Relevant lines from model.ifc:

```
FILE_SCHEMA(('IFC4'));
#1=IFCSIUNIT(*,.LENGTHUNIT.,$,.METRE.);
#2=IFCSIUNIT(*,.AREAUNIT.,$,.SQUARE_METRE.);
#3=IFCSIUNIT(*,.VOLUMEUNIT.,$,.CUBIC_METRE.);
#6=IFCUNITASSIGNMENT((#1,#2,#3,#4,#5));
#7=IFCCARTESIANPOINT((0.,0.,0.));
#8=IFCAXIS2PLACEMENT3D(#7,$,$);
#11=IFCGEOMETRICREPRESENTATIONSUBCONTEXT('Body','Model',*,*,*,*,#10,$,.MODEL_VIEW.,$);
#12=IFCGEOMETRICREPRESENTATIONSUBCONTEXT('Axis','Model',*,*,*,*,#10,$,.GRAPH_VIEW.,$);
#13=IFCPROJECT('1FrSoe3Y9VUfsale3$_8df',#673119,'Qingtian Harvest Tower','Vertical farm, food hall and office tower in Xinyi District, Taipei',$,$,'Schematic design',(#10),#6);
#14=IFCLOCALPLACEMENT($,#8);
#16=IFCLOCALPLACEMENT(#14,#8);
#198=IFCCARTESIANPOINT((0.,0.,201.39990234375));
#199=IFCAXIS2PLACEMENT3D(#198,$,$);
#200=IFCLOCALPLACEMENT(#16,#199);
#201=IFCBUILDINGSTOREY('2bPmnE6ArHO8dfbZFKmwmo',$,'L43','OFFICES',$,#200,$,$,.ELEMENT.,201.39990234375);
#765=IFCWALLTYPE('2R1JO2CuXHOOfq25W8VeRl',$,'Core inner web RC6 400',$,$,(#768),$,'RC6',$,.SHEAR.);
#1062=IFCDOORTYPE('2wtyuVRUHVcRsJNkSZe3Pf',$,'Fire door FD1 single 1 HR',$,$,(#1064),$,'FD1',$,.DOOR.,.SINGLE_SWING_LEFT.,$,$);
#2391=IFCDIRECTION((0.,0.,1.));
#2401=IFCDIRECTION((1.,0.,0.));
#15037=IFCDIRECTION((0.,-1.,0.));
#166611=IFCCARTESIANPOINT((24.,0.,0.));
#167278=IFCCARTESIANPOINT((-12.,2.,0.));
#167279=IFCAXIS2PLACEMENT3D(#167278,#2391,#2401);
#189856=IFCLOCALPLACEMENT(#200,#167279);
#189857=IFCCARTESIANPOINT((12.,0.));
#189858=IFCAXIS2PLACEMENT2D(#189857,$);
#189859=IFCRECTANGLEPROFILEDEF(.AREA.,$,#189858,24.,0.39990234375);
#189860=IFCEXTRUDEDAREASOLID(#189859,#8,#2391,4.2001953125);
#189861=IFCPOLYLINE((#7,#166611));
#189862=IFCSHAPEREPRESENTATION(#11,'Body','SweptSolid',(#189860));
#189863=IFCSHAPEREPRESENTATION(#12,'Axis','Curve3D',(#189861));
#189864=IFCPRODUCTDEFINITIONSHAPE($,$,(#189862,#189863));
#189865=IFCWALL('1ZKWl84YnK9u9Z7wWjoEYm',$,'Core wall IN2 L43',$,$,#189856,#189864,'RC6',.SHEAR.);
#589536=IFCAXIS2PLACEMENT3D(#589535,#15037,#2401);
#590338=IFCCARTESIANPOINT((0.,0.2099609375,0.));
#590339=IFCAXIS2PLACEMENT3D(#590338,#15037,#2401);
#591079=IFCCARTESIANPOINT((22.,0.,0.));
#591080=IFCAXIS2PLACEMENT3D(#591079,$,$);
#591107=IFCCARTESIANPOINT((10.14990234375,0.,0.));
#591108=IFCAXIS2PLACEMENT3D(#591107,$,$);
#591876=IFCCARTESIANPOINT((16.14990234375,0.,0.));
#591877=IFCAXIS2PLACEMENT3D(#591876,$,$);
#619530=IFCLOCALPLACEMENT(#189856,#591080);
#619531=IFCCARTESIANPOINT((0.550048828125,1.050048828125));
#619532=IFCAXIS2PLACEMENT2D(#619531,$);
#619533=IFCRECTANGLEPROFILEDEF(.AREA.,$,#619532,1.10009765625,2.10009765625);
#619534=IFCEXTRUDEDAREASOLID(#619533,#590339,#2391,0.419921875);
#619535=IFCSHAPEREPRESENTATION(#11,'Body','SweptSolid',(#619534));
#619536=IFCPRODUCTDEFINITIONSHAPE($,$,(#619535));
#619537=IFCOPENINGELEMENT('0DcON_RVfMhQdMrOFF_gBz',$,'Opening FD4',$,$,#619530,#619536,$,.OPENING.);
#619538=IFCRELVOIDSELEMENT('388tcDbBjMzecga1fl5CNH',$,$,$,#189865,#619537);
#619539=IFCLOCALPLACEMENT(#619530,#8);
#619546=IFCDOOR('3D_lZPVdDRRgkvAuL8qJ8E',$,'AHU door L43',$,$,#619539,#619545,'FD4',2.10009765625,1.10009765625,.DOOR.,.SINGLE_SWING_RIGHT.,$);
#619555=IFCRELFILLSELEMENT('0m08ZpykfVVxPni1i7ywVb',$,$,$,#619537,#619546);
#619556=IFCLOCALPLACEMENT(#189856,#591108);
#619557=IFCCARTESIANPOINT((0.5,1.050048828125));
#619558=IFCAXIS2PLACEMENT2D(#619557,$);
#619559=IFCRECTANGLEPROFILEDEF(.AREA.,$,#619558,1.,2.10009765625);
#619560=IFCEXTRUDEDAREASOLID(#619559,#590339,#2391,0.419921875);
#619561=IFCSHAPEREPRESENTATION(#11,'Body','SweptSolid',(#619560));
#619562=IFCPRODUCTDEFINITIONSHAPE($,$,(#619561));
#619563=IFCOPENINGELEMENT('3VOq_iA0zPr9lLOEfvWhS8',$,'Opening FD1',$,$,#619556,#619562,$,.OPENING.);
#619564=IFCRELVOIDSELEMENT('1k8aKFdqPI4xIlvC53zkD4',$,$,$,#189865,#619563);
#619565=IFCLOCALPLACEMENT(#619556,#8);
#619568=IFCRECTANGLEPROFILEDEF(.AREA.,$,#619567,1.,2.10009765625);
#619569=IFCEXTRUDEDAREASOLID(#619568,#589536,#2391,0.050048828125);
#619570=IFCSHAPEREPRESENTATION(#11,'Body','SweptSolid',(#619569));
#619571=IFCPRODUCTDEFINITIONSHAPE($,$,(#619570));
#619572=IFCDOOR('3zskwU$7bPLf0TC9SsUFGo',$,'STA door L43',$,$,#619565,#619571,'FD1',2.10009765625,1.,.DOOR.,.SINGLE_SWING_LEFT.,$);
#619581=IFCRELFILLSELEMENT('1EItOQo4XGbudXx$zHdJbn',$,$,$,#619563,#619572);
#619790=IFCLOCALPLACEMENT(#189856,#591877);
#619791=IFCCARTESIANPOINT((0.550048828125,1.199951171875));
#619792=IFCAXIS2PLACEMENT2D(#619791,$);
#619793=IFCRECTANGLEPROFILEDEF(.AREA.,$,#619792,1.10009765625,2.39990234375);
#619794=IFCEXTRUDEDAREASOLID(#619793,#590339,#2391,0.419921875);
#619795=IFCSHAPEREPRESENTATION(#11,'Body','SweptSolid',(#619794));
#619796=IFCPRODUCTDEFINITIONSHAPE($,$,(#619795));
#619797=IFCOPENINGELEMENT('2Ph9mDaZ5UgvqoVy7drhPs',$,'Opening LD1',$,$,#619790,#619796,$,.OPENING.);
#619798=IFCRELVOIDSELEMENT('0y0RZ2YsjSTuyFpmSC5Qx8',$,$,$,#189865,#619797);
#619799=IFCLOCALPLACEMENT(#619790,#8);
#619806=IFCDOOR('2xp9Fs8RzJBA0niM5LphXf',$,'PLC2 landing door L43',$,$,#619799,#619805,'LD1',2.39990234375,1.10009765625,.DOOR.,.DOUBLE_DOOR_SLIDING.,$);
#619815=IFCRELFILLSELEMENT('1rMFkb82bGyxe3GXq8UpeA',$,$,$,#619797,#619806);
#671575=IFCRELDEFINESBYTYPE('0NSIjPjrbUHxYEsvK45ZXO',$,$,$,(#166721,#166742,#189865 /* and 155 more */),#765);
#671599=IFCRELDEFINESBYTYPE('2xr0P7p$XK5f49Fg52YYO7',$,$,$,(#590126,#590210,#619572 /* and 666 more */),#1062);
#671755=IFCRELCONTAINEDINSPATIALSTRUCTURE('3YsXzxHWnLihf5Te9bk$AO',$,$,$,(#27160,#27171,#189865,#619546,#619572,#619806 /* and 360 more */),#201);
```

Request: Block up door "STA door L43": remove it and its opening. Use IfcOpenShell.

```python
import ifcopenshell
import ifcopenshell.api.feature
import ifcopenshell.api.root
import ifcopenshell.geom
import ifcopenshell.util.shape

model = ifcopenshell.open("model.ifc")
settings = ifcopenshell.geom.settings()


def volume(element):
    """Net volume in cubic metres, openings subtracted."""
    shape = ifcopenshell.geom.create_shape(settings, element)
    return ifcopenshell.util.shape.get_volume(shape.geometry)


door = model.by_guid("3zskwU$7bPLf0TC9SsUFGo")
opening = door.FillsVoids[0].RelatingOpeningElement
wall = opening.VoidsElements[0].RelatingBuildingElement
before = volume(wall)

ifcopenshell.api.root.remove_product(model, product=door)
ifcopenshell.api.feature.remove_feature(model, feature=opening)

after = volume(wall)

print(f"wall volume {before:.3f} -> {after:.3f} m3")

model.write("model_v2.ifc")
```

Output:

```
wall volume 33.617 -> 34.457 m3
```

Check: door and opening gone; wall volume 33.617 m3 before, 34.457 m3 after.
